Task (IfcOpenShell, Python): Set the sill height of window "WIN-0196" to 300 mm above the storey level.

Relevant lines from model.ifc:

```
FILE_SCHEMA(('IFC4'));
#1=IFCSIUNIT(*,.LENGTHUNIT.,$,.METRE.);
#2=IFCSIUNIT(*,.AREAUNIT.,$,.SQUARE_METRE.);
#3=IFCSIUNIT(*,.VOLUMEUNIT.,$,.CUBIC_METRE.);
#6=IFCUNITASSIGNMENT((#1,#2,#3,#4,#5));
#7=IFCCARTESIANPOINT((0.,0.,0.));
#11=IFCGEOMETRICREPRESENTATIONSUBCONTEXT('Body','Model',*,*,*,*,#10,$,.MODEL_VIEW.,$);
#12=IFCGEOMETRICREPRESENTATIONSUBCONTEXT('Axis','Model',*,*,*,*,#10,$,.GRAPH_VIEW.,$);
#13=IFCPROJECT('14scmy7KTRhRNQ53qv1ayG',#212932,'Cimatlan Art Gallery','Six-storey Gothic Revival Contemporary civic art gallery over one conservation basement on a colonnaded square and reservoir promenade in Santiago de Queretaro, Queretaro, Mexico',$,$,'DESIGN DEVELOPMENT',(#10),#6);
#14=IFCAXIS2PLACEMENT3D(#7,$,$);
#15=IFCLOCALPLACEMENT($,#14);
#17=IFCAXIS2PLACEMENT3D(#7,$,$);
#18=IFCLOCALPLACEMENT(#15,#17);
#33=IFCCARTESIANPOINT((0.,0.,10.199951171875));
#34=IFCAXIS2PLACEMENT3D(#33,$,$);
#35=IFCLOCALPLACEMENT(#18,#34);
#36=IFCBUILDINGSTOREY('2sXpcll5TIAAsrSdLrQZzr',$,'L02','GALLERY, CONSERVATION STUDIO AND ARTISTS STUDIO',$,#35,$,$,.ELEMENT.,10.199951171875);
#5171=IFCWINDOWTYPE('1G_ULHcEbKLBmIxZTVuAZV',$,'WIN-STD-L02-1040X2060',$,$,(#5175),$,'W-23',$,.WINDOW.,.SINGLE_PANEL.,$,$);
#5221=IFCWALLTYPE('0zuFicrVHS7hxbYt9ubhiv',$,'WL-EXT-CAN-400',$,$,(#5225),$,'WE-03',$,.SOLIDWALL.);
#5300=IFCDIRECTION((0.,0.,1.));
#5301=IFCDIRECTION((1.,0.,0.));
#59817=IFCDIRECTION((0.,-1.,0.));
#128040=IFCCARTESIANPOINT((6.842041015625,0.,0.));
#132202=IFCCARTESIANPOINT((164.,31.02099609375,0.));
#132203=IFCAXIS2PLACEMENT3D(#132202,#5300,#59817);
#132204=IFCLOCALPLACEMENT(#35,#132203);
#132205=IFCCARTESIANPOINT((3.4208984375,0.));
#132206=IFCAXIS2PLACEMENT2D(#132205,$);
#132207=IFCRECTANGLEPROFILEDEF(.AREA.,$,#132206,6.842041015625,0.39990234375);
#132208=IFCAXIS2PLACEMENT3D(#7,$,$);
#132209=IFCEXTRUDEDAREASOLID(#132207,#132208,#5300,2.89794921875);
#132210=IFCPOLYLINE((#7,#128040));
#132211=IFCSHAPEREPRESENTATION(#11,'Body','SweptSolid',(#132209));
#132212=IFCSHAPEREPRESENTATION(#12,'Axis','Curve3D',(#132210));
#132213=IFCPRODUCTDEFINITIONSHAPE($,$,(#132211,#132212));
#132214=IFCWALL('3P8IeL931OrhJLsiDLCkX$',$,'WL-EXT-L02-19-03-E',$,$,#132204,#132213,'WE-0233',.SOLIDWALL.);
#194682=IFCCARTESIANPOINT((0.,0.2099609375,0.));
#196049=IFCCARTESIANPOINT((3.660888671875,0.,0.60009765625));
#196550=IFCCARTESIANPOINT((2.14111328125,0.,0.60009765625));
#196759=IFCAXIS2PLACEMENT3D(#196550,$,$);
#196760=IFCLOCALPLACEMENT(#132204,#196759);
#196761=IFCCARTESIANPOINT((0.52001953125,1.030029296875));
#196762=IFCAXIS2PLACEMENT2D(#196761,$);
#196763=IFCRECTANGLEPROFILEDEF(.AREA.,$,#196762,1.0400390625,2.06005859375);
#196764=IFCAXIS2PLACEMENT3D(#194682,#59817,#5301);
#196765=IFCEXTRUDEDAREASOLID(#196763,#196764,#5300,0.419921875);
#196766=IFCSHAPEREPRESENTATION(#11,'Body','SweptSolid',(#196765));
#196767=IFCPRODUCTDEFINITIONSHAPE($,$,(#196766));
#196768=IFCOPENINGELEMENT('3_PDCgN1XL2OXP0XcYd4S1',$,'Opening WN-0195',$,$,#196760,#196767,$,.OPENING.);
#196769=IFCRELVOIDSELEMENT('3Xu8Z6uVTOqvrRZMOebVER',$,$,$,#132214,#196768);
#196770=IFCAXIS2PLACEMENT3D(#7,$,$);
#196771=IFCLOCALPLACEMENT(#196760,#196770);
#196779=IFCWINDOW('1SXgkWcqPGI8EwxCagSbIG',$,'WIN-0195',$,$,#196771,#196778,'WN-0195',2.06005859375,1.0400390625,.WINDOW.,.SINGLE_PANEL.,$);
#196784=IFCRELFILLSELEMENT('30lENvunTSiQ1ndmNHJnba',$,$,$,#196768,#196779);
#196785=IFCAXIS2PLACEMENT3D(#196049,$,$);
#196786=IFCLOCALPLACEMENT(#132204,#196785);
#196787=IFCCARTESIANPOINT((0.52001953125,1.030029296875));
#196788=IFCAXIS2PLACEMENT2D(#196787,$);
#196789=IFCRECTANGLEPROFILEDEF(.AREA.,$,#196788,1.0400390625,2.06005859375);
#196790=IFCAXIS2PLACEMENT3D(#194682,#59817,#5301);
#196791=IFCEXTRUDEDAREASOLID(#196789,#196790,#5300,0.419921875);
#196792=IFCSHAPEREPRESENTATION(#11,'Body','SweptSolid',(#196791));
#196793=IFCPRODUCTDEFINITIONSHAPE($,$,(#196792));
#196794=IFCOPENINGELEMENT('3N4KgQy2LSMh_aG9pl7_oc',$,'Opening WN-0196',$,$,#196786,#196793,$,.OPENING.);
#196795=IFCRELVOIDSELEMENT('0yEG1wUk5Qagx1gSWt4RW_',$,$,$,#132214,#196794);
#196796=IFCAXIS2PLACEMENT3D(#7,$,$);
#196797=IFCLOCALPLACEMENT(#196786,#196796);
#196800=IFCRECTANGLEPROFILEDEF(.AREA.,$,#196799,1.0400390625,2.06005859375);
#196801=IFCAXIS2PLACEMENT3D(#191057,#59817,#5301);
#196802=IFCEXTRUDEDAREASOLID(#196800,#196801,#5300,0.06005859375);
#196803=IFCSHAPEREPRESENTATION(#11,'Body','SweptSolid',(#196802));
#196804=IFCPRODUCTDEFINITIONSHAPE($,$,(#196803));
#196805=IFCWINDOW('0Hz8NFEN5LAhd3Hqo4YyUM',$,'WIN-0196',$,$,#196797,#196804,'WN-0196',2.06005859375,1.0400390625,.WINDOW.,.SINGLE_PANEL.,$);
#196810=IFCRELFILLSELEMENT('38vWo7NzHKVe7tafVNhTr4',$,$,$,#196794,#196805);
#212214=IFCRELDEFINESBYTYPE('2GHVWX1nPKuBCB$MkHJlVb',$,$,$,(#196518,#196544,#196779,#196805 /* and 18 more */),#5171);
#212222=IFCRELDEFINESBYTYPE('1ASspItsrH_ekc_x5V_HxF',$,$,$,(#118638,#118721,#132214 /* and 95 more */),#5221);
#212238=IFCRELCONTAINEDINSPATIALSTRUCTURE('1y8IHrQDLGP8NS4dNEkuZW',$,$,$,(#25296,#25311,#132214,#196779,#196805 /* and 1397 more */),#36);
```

```python
import numpy as np
import ifcopenshell
import ifcopenshell.api.geometry
import ifcopenshell.geom
import ifcopenshell.util.element
import ifcopenshell.util.placement
import ifcopenshell.util.shape
import ifcopenshell.util.unit

model = ifcopenshell.open("model.ifc")
unit_scale = ifcopenshell.util.unit.calculate_unit_scale(model)

window = model.by_guid("0Hz8NFEN5LAhd3Hqo4YyUM")
opening = window.FillsVoids[0].RelatingOpeningElement
storey = ifcopenshell.util.element.get_container(window, ifc_class="IfcBuildingStorey")
level = ifcopenshell.util.placement.get_local_placement(storey.ObjectPlacement)[2, 3]

# The opening's origin need not be at the sill, so measure its lowest point.
shape = ifcopenshell.geom.create_shape(ifcopenshell.geom.settings(), opening)
bottom = ifcopenshell.util.shape.get_shape_bottom_elevation(shape, shape.geometry) / unit_scale
dz = level + 0.3 / unit_scale - bottom

shift = np.array([0.0, 0.0, dz])
# The window is placed relative to its opening, so it follows when the opening moves.
matrix = ifcopenshell.util.placement.get_local_placement(opening.ObjectPlacement)
matrix[:3, 3] += shift
ifcopenshell.api.geometry.edit_object_placement(
    model, product=opening, matrix=matrix, is_si=False, should_transform_children=True
)

print(f"moved by {dz * unit_scale:+.3f} m")

model.write("model_v2.ifc")
```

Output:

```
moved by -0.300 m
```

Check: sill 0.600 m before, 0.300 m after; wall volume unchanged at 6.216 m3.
